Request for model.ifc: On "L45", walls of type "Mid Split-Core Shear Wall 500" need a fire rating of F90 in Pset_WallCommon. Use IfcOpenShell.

First a look at what the model holds.

```python
import ifcopenshell
import ifcopenshell.util.element

model = ifcopenshell.open("model.ifc")
print(model.schema)
storey = next(s for s in model.by_type("IfcBuildingStorey") if s.Name == "L45")
walls = [e for e in ifcopenshell.util.element.get_decomposition(storey) if e.is_a("IfcWall")]
seen = {}
for e in walls:
    element_type = ifcopenshell.util.element.get_type(e)
    key = (element_type.Name if element_type != e and element_type else None, ifcopenshell.util.element.get_pset(e, "Pset_WallCommon", "FireRating"))
    seen[key] = seen.get(key, 0) + 1
for (name, value), count in sorted(seen.items(), key=str):
    print(count, "x", name, "|", value)
```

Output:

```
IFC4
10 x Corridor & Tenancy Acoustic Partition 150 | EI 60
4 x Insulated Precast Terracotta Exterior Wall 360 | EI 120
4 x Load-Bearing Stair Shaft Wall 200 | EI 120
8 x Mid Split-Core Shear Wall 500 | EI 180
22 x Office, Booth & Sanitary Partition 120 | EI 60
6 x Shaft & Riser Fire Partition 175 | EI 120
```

```python
import ifcopenshell
import ifcopenshell.api.pset
import ifcopenshell.util.element

model = ifcopenshell.open("model.ifc")

storey = next(s for s in model.by_type("IfcBuildingStorey") if s.Name == "L45")
walls = [e for e in ifcopenshell.util.element.get_decomposition(storey) if e.is_a("IfcWall")]

count = 0
for e in walls:
    element_type = ifcopenshell.util.element.get_type(e)
    if element_type in (None, e) or element_type.Name != "Mid Split-Core Shear Wall 500":
        continue
    found = ifcopenshell.util.element.get_pset(e, "Pset_WallCommon", should_inherit=False)
    if found:
        pset = model.by_id(found["id"])
        if len(ifcopenshell.util.element.get_elements_by_pset(pset)) > 1:
            pset = ifcopenshell.api.pset.unshare_pset(model, products=[e], pset=pset)[0]
    else:
        pset = ifcopenshell.api.pset.add_pset(model, product=e, name="Pset_WallCommon")
    ifcopenshell.api.pset.edit_pset(model, pset=pset, properties={"FireRating": "F90"})
    count += 1

print(count, "walls updated")

model.write("model_updated.ifc")
```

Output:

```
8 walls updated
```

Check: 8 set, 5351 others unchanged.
